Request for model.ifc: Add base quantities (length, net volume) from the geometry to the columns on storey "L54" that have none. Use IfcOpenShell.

First a look at what the model holds.

```python
import ifcopenshell
import ifcopenshell.util.element
import ifcopenshell.util.unit

model = ifcopenshell.open("model.ifc")
print(model.schema)
for unit_type in ("LENGTHUNIT", "AREAUNIT", "VOLUMEUNIT"):
    print(unit_type, ifcopenshell.util.unit.calculate_unit_scale(model, unit_type))
storey = next(s for s in model.by_type("IfcBuildingStorey") if s.Name == "L54")
columns = [e for e in ifcopenshell.util.element.get_decomposition(storey) if e.is_a("IfcColumn")]
for e in sorted(columns, key=lambda e: e.id()):
    print(e.id(), e.is_a(), e.Name, list(ifcopenshell.util.element.get_psets(e, qtos_only=True)), sep=" | ")
```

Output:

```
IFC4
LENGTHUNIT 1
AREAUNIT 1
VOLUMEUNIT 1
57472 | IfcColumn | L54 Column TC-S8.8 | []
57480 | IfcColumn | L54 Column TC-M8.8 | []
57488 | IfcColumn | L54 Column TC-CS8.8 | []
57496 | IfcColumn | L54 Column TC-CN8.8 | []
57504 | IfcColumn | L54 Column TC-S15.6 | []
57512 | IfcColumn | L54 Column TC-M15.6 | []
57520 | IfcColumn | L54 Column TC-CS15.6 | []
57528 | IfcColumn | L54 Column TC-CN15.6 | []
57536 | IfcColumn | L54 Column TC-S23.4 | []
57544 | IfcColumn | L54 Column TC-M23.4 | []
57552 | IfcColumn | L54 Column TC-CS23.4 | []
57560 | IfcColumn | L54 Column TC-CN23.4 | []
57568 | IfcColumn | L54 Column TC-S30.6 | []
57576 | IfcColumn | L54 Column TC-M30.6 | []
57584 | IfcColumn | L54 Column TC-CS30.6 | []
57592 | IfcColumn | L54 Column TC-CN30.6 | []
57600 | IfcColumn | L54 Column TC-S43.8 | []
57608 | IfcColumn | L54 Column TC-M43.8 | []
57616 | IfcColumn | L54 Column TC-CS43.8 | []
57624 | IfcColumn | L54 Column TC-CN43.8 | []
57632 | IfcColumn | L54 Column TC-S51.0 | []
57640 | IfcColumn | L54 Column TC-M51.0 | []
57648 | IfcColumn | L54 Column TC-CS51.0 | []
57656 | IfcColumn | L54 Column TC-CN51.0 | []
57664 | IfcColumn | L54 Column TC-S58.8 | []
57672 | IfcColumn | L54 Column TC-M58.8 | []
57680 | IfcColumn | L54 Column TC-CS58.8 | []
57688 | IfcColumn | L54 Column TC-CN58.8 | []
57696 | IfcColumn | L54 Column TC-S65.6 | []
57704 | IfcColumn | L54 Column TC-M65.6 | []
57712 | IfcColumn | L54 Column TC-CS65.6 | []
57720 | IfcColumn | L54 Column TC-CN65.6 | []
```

```python
import ifcopenshell
import ifcopenshell.api.pset
import ifcopenshell.geom
import ifcopenshell.util.element
import ifcopenshell.util.shape
import ifcopenshell.util.unit

model = ifcopenshell.open("model.ifc")
unit_scale = ifcopenshell.util.unit.calculate_unit_scale(model)
volume_scale = ifcopenshell.util.unit.calculate_unit_scale(model, "VOLUMEUNIT")
settings = ifcopenshell.geom.settings()

storey = next(s for s in model.by_type("IfcBuildingStorey") if s.Name == "L54")
columns = [e for e in ifcopenshell.util.element.get_decomposition(storey) if e.is_a("IfcColumn")]

for e in sorted(columns, key=lambda e: e.id()):
    if ifcopenshell.util.element.get_psets(e, qtos_only=True, should_inherit=False):
        continue
    # Geometry comes back in metres, in the element's own axes.
    shape = ifcopenshell.geom.create_shape(settings, e)
    values = {
        "Length": ifcopenshell.util.shape.get_z(shape.geometry) / unit_scale,
        "NetVolume": ifcopenshell.util.shape.get_volume(shape.geometry) / volume_scale,
    }
    qto = ifcopenshell.api.pset.add_qto(model, product=e, name="Qto_ColumnBaseQuantities")
    ifcopenshell.api.pset.edit_qto(model, qto=qto, properties=values)
    print(e.id(), {k: round(v, 3) for k, v in values.items()})

model.write("model_rev.ifc")
```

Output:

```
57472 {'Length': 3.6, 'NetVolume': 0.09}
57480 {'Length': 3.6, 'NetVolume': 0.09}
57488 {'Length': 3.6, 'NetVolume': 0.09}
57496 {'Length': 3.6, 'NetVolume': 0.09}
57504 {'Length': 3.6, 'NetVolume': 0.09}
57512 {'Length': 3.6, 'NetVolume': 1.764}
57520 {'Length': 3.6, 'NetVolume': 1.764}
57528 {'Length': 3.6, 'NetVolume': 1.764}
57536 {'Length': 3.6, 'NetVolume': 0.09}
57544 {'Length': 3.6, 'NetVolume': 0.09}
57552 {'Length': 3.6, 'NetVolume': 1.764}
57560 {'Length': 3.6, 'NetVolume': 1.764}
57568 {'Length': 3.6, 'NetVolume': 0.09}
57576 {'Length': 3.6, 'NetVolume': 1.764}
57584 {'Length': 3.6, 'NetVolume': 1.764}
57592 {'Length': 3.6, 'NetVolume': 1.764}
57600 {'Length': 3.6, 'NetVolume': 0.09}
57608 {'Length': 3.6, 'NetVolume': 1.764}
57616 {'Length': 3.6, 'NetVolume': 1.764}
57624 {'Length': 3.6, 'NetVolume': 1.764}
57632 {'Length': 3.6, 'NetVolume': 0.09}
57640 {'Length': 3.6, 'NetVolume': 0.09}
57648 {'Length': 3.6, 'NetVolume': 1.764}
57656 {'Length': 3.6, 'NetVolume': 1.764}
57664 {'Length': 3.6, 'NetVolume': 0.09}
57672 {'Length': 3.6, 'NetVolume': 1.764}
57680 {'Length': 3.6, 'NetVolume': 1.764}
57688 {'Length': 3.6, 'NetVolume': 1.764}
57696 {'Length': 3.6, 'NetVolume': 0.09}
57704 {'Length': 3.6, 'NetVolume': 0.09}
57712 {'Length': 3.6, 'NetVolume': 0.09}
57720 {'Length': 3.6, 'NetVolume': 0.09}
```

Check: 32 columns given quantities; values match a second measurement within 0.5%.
